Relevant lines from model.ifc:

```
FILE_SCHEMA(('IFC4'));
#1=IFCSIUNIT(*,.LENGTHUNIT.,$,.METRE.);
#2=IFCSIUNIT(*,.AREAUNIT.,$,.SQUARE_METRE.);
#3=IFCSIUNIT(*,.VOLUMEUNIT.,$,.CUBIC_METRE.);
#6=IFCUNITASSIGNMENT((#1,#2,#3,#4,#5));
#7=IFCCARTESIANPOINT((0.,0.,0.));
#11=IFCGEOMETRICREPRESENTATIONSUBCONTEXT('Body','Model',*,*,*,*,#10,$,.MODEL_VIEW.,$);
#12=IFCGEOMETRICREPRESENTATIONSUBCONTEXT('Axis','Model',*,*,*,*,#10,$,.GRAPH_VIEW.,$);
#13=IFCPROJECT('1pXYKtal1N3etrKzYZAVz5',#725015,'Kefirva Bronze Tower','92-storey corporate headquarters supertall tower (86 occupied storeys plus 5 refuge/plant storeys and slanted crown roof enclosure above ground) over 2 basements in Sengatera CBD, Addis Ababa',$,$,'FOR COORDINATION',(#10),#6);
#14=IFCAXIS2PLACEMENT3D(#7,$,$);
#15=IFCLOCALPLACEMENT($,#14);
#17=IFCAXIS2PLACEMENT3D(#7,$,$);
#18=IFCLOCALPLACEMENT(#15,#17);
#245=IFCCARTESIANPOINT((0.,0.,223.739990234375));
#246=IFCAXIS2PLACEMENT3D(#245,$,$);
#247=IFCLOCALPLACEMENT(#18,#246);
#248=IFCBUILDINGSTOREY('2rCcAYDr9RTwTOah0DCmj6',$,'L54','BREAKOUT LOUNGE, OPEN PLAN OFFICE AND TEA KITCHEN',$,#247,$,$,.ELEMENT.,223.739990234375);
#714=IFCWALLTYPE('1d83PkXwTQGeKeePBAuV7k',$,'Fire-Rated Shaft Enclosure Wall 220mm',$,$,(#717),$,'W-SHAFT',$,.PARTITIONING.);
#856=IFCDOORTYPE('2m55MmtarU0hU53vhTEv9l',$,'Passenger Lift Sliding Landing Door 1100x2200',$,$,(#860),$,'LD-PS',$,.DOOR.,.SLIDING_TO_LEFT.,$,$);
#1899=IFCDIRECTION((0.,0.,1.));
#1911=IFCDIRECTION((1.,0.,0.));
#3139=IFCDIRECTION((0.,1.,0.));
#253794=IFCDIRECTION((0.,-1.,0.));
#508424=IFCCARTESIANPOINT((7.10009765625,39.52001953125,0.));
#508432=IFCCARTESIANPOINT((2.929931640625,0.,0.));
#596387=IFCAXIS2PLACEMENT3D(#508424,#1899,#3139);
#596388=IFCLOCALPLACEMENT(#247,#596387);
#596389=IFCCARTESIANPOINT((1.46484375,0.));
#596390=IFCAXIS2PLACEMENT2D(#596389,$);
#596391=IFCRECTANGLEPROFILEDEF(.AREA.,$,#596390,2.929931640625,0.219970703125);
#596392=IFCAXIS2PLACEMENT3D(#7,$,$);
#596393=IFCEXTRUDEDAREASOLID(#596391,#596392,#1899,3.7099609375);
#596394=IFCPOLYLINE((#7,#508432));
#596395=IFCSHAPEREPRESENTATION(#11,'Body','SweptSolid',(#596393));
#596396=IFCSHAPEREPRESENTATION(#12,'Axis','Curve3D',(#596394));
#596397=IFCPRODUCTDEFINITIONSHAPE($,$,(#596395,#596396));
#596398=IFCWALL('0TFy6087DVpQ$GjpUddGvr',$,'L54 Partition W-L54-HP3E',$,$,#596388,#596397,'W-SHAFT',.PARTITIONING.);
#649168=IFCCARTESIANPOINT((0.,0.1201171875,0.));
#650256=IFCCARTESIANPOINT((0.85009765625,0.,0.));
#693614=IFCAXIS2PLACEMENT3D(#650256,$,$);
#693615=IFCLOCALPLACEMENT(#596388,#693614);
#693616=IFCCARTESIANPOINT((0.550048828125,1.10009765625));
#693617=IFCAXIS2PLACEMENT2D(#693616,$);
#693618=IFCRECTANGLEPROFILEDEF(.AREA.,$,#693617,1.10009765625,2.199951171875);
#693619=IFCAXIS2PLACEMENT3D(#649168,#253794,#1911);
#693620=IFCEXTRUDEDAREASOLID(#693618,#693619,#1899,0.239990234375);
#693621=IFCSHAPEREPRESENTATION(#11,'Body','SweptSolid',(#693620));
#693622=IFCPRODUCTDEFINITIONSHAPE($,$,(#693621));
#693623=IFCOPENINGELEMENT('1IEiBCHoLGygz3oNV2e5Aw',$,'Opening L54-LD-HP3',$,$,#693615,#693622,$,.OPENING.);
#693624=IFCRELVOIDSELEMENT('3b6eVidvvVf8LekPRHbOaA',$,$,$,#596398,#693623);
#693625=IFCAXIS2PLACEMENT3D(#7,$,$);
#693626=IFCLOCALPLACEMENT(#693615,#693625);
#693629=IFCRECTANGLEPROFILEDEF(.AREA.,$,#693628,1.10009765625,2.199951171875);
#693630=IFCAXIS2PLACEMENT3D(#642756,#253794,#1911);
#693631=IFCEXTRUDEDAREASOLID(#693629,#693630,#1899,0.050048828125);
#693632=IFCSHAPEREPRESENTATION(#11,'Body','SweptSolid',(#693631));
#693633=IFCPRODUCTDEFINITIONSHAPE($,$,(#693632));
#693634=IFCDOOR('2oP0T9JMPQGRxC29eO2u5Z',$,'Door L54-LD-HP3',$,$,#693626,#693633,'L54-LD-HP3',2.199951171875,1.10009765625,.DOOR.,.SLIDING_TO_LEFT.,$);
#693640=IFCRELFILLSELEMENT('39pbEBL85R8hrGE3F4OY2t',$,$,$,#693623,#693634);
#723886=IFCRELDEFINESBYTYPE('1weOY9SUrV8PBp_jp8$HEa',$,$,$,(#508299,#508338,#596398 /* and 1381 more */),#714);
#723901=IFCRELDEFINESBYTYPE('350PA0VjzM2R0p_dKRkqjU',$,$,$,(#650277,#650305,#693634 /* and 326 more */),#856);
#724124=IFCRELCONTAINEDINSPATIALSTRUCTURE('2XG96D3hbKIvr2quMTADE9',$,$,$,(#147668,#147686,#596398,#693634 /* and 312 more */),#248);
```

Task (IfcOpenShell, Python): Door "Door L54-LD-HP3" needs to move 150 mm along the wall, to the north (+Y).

```python
import ifcopenshell
import ifcopenshell.api.geometry
import ifcopenshell.util.placement

model = ifcopenshell.open("model.ifc")

door = model.by_id(693634)
opening = door.FillsVoids[0].RelatingOpeningElement
wall = opening.VoidsElements[0].RelatingBuildingElement

wall_matrix = ifcopenshell.util.placement.get_local_placement(wall.ObjectPlacement)
shift = wall_matrix[:3, 0] * 0.15
before = ifcopenshell.util.placement.get_local_placement(door.ObjectPlacement)[:3, 3].copy()

# The door is placed relative to its opening, so it follows when the opening moves.
matrix = ifcopenshell.util.placement.get_local_placement(opening.ObjectPlacement)
matrix[:3, 3] += shift
ifcopenshell.api.geometry.edit_object_placement(
    model, product=opening, matrix=matrix, is_si=False, should_transform_children=True
)

after = ifcopenshell.util.placement.get_local_placement(door.ObjectPlacement)[:3, 3]
print("door moved by", (after - before).round(3) + 0.0)

model.write("model_rev.ifc")
```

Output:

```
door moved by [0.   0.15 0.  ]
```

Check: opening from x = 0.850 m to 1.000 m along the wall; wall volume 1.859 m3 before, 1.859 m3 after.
